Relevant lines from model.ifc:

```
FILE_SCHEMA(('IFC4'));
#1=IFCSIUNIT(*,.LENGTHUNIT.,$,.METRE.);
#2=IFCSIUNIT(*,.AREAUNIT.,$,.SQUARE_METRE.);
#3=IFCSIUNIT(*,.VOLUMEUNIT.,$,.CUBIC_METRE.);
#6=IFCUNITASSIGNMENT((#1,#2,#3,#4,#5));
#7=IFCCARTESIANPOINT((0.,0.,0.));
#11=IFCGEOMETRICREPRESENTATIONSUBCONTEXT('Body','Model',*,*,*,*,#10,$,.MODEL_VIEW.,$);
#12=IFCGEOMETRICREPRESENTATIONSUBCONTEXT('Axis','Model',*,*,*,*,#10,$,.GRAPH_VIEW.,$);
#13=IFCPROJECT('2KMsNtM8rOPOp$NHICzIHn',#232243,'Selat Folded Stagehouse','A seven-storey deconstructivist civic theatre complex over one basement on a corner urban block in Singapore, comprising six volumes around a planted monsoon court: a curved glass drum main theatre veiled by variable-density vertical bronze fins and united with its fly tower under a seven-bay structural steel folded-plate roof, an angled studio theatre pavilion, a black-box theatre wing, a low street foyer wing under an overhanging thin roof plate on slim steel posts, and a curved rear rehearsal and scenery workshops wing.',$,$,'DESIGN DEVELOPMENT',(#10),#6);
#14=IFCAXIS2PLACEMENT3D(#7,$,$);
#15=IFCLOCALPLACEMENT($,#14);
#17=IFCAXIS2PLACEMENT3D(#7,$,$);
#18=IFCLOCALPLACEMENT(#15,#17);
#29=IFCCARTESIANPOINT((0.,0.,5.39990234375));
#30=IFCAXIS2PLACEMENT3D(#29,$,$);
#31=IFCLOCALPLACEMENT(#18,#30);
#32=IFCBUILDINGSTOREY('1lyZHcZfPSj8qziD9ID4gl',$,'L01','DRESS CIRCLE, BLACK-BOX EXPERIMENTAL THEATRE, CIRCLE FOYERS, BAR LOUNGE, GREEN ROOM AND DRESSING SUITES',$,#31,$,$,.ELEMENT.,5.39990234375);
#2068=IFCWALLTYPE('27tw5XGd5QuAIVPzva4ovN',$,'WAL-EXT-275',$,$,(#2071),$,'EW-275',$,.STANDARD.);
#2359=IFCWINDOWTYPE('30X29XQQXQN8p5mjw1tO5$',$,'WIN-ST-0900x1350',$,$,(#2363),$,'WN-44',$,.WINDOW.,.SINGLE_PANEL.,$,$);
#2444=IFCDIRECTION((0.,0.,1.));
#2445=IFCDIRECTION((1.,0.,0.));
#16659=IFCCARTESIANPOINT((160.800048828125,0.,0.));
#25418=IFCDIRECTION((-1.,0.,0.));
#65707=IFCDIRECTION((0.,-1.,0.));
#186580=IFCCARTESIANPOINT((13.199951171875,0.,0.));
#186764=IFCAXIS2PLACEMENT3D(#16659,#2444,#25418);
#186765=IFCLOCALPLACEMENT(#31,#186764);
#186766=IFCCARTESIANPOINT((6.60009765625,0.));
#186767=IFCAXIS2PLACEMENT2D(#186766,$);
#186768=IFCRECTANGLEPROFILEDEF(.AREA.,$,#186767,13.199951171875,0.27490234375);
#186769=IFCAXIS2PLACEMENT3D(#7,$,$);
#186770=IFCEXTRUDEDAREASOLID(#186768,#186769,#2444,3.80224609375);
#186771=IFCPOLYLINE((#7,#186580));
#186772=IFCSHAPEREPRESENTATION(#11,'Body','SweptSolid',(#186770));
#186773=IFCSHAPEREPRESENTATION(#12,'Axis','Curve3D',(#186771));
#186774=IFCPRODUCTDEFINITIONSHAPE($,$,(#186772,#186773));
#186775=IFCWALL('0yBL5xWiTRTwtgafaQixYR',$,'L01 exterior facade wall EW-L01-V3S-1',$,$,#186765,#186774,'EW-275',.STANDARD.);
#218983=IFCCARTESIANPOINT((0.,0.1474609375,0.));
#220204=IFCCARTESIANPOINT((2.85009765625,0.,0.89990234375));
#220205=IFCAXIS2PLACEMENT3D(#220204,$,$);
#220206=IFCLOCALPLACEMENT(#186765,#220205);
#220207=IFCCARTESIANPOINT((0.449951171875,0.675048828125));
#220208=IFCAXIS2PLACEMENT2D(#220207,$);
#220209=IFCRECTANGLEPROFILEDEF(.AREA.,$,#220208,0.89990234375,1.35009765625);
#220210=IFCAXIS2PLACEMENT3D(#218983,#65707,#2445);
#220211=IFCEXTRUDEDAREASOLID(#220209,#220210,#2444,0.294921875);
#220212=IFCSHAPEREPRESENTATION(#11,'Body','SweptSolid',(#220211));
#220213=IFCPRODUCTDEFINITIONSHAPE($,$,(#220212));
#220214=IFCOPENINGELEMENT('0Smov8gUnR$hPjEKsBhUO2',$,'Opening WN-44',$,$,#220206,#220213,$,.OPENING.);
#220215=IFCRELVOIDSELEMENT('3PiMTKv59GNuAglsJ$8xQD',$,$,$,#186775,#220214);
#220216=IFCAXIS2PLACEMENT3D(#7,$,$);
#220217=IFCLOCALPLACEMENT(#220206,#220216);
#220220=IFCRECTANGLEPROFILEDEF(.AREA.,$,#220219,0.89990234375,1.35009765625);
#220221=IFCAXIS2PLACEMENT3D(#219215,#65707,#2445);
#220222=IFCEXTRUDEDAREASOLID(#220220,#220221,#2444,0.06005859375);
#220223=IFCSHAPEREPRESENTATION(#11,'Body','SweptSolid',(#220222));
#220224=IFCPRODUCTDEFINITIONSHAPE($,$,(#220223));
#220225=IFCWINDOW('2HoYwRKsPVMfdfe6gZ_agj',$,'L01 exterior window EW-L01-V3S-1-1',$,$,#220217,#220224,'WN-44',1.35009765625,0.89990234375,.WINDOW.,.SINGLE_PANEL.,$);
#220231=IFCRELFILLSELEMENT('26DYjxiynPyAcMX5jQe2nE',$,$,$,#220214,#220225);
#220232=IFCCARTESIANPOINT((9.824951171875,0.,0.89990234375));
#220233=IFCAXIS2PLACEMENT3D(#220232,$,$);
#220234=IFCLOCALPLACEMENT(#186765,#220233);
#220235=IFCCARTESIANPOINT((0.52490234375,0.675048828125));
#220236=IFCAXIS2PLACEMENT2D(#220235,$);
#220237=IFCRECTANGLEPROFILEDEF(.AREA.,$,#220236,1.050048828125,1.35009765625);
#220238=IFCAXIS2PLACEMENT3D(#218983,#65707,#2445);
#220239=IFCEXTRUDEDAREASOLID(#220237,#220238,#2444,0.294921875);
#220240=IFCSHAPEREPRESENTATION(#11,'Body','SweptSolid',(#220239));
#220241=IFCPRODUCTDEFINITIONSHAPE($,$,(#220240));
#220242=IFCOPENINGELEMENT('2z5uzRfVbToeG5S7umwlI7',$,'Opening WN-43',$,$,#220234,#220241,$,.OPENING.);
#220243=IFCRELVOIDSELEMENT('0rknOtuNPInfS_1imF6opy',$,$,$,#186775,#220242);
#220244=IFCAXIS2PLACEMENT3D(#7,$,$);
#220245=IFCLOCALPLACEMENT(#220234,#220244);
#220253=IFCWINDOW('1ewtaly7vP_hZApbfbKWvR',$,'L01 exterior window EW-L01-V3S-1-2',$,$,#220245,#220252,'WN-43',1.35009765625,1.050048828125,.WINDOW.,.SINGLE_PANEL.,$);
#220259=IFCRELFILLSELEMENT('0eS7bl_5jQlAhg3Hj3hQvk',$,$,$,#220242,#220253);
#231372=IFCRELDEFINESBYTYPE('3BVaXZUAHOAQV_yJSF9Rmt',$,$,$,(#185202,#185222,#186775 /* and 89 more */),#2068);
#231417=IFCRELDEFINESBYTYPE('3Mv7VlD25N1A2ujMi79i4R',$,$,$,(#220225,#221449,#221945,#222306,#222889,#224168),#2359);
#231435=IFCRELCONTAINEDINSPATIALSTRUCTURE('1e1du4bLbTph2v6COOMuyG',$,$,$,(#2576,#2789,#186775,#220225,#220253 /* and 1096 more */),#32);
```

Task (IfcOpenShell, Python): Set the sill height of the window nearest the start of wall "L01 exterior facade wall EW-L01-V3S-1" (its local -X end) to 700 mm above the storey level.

```python
import numpy as np
import ifcopenshell
import ifcopenshell.api.geometry
import ifcopenshell.geom
import ifcopenshell.util.element
import ifcopenshell.util.placement
import ifcopenshell.util.shape
import ifcopenshell.util.unit

model = ifcopenshell.open("model.ifc")
unit_scale = ifcopenshell.util.unit.calculate_unit_scale(model)

window = model.by_guid("2HoYwRKsPVMfdfe6gZ_agj")
opening = window.FillsVoids[0].RelatingOpeningElement
storey = ifcopenshell.util.element.get_container(window, ifc_class="IfcBuildingStorey")
level = ifcopenshell.util.placement.get_local_placement(storey.ObjectPlacement)[2, 3]

# The opening's origin need not be at the sill, so measure its lowest point.
shape = ifcopenshell.geom.create_shape(ifcopenshell.geom.settings(), opening)
bottom = ifcopenshell.util.shape.get_shape_bottom_elevation(shape, shape.geometry) / unit_scale
dz = level + 0.7 - bottom

shift = np.array([0.0, 0.0, dz])
# The window is placed relative to its opening, so it follows when the opening moves.
matrix = ifcopenshell.util.placement.get_local_placement(opening.ObjectPlacement)
matrix[:3, 3] += shift
ifcopenshell.api.geometry.edit_object_placement(
    model, product=opening, matrix=matrix, is_si=False, should_transform_children=True
)

print(f"moved by {dz * unit_scale:+.3f} m")

model.write("model_edited.ifc")
```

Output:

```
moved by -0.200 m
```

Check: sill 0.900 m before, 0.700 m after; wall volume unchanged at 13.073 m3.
